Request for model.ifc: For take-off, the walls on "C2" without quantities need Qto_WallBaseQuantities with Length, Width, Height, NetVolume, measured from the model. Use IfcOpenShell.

First a look at what the model holds.

```python
import ifcopenshell
import ifcopenshell.util.element
import ifcopenshell.util.unit

model = ifcopenshell.open("model.ifc")
print(model.schema)
for unit_type in ("LENGTHUNIT", "AREAUNIT", "VOLUMEUNIT"):
    print(unit_type, ifcopenshell.util.unit.calculate_unit_scale(model, unit_type))
storey = next(s for s in model.by_type("IfcBuildingStorey") if s.Name == "C2")
walls = [e for e in ifcopenshell.util.element.get_decomposition(storey) if e.is_a("IfcWall")]
for e in sorted(walls, key=lambda e: e.id()):
    print(e.id(), e.is_a(), e.Name, list(ifcopenshell.util.element.get_psets(e, qtos_only=True)), sep=" | ")
```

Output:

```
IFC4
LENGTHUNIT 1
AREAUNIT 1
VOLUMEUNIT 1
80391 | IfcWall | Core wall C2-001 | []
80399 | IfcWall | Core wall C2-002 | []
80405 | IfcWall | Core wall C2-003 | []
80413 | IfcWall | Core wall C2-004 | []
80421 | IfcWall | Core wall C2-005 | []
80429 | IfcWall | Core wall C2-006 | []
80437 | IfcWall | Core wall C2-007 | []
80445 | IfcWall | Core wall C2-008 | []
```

```python
import ifcopenshell
import ifcopenshell.api.pset
import ifcopenshell.geom
import ifcopenshell.util.element
import ifcopenshell.util.shape
import ifcopenshell.util.unit

model = ifcopenshell.open("model.ifc")
unit_scale = ifcopenshell.util.unit.calculate_unit_scale(model)
volume_scale = ifcopenshell.util.unit.calculate_unit_scale(model, "VOLUMEUNIT")
settings = ifcopenshell.geom.settings()

storey = next(s for s in model.by_type("IfcBuildingStorey") if s.Name == "C2")
walls = [e for e in ifcopenshell.util.element.get_decomposition(storey) if e.is_a("IfcWall")]

for e in sorted(walls, key=lambda e: e.id()):
    if ifcopenshell.util.element.get_psets(e, qtos_only=True, should_inherit=False):
        continue
    # Geometry comes back in metres, in the element's own axes.
    shape = ifcopenshell.geom.create_shape(settings, e)
    values = {
        "Length": ifcopenshell.util.shape.get_x(shape.geometry) / unit_scale,
        "Width": ifcopenshell.util.shape.get_y(shape.geometry) / unit_scale,
        "Height": ifcopenshell.util.shape.get_z(shape.geometry) / unit_scale,
        "NetVolume": ifcopenshell.util.shape.get_volume(shape.geometry) / volume_scale,
    }
    qto = ifcopenshell.api.pset.add_qto(model, product=e, name="Qto_WallBaseQuantities")
    ifcopenshell.api.pset.edit_qto(model, qto=qto, properties=values)
    print(e.id(), {k: round(v, 3) for k, v in values.items()})

model.write("model_updated.ifc")
```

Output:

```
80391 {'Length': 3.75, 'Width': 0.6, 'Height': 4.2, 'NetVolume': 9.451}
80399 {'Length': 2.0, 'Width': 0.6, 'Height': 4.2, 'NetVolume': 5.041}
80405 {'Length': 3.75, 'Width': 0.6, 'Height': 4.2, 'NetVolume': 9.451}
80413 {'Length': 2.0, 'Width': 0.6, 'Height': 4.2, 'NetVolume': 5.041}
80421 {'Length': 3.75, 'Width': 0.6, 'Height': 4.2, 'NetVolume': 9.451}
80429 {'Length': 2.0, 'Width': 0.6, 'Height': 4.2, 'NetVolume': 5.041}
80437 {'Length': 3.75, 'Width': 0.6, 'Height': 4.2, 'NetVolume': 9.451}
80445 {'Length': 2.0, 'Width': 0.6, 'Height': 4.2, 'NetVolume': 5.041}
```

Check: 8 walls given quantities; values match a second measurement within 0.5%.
